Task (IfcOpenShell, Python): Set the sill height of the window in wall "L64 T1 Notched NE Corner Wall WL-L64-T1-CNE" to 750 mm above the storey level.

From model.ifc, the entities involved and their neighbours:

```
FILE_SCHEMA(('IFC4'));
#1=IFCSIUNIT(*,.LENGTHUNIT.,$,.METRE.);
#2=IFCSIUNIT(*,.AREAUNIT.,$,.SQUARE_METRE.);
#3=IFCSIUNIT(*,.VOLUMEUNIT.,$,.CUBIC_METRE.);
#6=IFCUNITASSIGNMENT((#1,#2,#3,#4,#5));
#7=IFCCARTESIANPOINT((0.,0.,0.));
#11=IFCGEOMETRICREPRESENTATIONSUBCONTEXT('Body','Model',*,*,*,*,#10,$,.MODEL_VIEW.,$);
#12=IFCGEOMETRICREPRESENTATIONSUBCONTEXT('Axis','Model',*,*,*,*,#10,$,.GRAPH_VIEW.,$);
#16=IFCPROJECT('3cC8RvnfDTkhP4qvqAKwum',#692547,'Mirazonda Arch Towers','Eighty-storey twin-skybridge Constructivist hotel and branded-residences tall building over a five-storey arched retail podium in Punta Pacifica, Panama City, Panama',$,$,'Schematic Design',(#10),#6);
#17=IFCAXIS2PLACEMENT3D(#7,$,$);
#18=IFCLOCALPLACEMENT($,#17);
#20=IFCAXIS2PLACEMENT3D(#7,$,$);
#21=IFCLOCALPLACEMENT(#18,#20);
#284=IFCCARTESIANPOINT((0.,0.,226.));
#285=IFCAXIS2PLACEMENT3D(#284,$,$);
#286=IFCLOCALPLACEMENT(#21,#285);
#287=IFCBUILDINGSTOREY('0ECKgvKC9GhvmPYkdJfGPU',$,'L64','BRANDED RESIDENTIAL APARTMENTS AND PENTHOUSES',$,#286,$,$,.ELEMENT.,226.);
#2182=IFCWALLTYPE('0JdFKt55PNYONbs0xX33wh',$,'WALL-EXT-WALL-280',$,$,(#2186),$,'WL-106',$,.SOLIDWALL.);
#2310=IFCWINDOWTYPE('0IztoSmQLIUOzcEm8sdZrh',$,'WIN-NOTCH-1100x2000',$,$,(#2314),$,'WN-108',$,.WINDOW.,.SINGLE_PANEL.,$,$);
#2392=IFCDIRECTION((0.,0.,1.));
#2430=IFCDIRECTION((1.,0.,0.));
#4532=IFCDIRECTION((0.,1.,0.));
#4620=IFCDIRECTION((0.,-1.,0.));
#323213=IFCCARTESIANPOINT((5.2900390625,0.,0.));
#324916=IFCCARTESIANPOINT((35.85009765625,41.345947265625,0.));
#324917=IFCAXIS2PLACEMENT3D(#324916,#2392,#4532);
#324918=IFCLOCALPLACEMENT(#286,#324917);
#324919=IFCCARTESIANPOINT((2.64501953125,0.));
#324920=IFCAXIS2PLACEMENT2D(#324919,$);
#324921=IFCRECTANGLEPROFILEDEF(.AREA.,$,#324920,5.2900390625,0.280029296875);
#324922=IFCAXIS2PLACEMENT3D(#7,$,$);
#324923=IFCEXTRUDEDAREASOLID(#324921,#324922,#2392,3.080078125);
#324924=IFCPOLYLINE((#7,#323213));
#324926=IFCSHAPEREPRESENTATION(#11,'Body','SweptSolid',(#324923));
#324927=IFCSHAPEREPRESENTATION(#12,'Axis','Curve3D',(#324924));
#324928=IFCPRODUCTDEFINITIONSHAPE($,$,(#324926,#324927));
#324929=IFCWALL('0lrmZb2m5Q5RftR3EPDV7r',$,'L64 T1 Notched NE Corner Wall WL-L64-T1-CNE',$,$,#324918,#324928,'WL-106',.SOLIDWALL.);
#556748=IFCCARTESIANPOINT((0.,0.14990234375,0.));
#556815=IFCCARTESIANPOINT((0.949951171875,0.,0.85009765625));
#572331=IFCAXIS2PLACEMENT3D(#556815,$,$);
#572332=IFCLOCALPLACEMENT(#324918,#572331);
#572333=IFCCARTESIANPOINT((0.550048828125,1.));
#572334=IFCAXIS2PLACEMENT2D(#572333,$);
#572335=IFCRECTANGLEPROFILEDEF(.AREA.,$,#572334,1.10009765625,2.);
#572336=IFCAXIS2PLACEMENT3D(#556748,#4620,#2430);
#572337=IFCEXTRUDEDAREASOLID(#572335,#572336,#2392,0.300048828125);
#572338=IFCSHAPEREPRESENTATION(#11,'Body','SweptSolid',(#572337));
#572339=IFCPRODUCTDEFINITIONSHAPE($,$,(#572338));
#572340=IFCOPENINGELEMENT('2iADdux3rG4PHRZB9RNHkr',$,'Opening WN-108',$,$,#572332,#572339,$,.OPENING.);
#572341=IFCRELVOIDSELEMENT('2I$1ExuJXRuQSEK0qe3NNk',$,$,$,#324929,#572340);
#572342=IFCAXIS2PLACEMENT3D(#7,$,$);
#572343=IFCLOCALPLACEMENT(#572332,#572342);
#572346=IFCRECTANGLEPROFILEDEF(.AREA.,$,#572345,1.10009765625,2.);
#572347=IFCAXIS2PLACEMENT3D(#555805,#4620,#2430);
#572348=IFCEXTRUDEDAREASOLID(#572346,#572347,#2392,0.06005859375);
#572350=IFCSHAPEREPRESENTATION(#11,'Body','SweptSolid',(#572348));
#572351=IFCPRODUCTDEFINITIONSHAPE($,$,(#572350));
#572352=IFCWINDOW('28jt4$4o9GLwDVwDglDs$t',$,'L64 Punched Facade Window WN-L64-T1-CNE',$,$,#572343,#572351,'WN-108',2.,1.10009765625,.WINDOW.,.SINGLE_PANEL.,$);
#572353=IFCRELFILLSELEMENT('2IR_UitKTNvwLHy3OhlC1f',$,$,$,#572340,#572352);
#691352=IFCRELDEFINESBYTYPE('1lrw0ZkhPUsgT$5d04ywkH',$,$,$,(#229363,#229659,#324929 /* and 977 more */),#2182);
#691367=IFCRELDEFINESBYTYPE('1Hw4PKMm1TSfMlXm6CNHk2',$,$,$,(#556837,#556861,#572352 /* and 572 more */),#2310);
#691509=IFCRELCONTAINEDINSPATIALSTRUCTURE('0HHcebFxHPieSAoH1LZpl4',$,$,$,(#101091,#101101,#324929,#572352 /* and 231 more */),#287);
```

```python
import numpy as np
import ifcopenshell
import ifcopenshell.api.geometry
import ifcopenshell.geom
import ifcopenshell.util.element
import ifcopenshell.util.placement
import ifcopenshell.util.shape
import ifcopenshell.util.unit

model = ifcopenshell.open("model.ifc")
unit_scale = ifcopenshell.util.unit.calculate_unit_scale(model)

window = model.by_guid("28jt4$4o9GLwDVwDglDs$t")
opening = window.FillsVoids[0].RelatingOpeningElement
storey = ifcopenshell.util.element.get_container(window, ifc_class="IfcBuildingStorey")
level = ifcopenshell.util.placement.get_local_placement(storey.ObjectPlacement)[2, 3]

# The opening's origin need not be at the sill, so measure its lowest point.
shape = ifcopenshell.geom.create_shape(ifcopenshell.geom.settings(), opening)
bottom = ifcopenshell.util.shape.get_shape_bottom_elevation(shape, shape.geometry) / unit_scale
dz = level + 0.75 / unit_scale - bottom

shift = np.array([0.0, 0.0, dz])
# The window is placed relative to its opening, so it follows when the opening moves.
matrix = ifcopenshell.util.placement.get_local_placement(opening.ObjectPlacement)
matrix[:3, 3] += shift
ifcopenshell.api.geometry.edit_object_placement(
    model, product=opening, matrix=matrix, is_si=False, should_transform_children=True
)

print(f"moved by {dz * unit_scale:+.3f} m")

model.write("model_rev.ifc")
```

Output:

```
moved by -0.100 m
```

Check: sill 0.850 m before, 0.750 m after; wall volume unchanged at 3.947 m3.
